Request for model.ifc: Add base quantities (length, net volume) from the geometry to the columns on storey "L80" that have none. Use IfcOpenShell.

First a look at what the model holds.

```python
import ifcopenshell
import ifcopenshell.util.element
import ifcopenshell.util.unit

model = ifcopenshell.open("model.ifc")
print(model.schema)
for unit_type in ("LENGTHUNIT", "AREAUNIT", "VOLUMEUNIT"):
    print(unit_type, ifcopenshell.util.unit.calculate_unit_scale(model, unit_type))
storey = next(s for s in model.by_type("IfcBuildingStorey") if s.Name == "L80")
columns = [e for e in ifcopenshell.util.element.get_decomposition(storey) if e.is_a("IfcColumn")]
for e in sorted(columns, key=lambda e: e.id()):
    print(e.id(), e.is_a(), e.Name, list(ifcopenshell.util.element.get_psets(e, qtos_only=True)), sep=" | ")
```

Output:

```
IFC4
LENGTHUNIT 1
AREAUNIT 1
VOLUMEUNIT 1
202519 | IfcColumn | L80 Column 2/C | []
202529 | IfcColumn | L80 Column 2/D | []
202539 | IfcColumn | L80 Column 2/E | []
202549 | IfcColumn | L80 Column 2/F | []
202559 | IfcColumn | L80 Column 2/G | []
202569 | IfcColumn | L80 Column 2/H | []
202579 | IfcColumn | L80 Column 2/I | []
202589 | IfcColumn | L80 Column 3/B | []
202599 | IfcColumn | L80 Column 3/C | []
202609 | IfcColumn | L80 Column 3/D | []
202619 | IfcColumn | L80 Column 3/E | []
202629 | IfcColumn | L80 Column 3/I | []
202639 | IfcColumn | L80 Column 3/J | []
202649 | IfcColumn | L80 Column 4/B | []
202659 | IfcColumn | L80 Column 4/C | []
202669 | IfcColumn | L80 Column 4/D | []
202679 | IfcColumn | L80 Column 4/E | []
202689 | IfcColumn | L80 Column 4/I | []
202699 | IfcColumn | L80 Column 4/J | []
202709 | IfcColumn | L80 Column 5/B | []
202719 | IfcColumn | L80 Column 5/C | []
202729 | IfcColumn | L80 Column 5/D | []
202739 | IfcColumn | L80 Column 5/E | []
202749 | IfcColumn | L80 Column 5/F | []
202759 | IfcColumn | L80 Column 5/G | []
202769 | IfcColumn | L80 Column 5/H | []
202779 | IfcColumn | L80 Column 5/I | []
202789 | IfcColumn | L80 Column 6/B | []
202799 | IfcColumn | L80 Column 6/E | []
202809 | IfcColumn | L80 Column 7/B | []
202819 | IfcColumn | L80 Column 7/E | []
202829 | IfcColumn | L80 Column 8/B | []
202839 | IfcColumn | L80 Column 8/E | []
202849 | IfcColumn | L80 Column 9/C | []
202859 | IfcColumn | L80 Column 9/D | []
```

```python
import ifcopenshell
import ifcopenshell.api.pset
import ifcopenshell.geom
import ifcopenshell.util.element
import ifcopenshell.util.shape
import ifcopenshell.util.unit

model = ifcopenshell.open("model.ifc")
unit_scale = ifcopenshell.util.unit.calculate_unit_scale(model)
volume_scale = ifcopenshell.util.unit.calculate_unit_scale(model, "VOLUMEUNIT")
settings = ifcopenshell.geom.settings()

storey = next(s for s in model.by_type("IfcBuildingStorey") if s.Name == "L80")
columns = [e for e in ifcopenshell.util.element.get_decomposition(storey) if e.is_a("IfcColumn")]

for e in sorted(columns, key=lambda e: e.id()):
    if ifcopenshell.util.element.get_psets(e, qtos_only=True, should_inherit=False):
        continue
    # Geometry comes back in metres, in the element's own axes.
    shape = ifcopenshell.geom.create_shape(settings, e)
    values = {
        "Length": ifcopenshell.util.shape.get_z(shape.geometry) / unit_scale,
        "NetVolume": ifcopenshell.util.shape.get_volume(shape.geometry) / volume_scale,
    }
    qto = ifcopenshell.api.pset.add_qto(model, product=e, name="Qto_ColumnBaseQuantities")
    ifcopenshell.api.pset.edit_qto(model, qto=qto, properties=values)
    print(e.id(), {k: round(v, 3) for k, v in values.items()})

model.write("model_edited.ifc")
```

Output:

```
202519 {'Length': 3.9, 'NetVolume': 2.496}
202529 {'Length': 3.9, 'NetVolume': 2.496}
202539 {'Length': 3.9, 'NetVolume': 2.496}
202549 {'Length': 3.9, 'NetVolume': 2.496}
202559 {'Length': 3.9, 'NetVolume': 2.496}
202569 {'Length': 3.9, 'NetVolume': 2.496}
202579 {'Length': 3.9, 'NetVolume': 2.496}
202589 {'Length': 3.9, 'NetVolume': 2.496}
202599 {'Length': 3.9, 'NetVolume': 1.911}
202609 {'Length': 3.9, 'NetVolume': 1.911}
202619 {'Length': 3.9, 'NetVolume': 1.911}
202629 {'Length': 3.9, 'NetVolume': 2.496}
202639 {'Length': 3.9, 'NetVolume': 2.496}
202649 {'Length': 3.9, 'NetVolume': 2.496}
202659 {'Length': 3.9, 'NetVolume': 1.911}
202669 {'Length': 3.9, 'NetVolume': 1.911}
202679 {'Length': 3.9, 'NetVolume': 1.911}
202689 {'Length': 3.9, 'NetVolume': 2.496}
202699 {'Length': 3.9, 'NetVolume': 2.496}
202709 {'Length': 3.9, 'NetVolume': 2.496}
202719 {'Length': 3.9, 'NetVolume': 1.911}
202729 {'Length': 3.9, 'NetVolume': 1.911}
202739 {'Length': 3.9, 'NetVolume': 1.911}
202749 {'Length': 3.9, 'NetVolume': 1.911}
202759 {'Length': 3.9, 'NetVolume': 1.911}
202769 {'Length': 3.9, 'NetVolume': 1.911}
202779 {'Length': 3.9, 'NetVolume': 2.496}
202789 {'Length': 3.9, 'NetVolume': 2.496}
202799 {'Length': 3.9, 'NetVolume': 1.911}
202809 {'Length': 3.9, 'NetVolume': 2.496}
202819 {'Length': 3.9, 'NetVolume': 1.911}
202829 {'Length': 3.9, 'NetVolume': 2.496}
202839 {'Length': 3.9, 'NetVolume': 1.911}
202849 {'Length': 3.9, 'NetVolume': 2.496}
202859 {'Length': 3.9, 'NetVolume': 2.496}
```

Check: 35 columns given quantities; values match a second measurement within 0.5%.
